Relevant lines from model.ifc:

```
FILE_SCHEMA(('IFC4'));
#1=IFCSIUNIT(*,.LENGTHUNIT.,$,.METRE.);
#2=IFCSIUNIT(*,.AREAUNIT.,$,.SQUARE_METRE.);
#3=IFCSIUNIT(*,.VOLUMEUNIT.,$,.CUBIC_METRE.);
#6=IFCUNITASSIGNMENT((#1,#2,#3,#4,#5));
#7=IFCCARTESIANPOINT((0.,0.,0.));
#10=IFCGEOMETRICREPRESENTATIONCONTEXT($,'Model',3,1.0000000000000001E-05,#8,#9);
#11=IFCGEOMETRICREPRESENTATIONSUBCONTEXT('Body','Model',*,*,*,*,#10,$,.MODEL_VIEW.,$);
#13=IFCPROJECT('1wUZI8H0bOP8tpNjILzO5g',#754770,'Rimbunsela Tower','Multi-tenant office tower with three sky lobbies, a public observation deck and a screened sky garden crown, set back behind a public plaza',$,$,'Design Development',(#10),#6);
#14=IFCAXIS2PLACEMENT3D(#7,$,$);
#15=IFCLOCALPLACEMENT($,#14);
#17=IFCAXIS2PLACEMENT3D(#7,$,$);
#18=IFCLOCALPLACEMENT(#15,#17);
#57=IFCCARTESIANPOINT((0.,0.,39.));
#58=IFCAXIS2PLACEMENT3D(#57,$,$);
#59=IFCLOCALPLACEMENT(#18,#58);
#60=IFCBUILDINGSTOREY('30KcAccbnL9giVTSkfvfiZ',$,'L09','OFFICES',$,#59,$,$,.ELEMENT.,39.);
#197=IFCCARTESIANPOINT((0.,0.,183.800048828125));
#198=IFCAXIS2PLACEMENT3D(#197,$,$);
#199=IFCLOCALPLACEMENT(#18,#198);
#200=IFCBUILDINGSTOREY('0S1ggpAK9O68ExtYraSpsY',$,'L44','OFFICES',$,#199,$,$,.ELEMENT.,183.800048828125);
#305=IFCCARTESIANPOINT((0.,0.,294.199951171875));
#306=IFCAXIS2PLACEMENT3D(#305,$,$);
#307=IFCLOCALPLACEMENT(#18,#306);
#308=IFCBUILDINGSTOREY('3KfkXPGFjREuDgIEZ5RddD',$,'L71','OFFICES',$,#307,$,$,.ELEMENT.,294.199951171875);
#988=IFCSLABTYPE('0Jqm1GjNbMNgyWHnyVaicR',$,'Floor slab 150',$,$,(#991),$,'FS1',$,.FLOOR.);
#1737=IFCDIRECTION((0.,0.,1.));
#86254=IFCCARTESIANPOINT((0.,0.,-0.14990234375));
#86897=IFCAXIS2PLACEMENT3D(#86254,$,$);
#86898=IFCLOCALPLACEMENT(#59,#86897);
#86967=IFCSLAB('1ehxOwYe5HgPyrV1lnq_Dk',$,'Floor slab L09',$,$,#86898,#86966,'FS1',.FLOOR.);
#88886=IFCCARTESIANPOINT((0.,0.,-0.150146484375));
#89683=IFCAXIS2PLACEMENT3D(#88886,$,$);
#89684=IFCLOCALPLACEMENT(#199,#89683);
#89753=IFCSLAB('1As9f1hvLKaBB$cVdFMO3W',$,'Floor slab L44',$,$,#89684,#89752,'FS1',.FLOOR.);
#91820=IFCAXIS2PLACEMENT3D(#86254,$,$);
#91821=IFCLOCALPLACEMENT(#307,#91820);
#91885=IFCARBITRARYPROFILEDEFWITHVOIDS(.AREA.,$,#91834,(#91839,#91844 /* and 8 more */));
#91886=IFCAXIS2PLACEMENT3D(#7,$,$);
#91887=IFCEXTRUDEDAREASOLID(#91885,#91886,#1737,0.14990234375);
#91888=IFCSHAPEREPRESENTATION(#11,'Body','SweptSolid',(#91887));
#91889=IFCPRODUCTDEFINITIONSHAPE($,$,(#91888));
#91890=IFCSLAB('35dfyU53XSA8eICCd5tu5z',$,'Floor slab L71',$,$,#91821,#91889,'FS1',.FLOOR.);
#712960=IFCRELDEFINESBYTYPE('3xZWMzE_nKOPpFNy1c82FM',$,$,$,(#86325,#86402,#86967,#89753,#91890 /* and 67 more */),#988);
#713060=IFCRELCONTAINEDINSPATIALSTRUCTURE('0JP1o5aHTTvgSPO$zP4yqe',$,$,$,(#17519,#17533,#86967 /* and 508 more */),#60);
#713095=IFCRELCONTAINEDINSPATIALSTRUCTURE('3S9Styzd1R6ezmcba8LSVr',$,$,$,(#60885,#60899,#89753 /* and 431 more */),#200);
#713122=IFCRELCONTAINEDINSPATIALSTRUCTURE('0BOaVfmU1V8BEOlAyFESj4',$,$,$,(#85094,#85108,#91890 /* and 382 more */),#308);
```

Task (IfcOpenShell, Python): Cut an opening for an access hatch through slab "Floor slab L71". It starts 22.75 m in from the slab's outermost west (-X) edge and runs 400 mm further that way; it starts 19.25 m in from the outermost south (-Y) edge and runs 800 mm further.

```python
import numpy as np
import ifcopenshell
import ifcopenshell.api.feature
import ifcopenshell.api.geometry
import ifcopenshell.api.root
import ifcopenshell.geom
import ifcopenshell.util.placement
import ifcopenshell.util.representation
import ifcopenshell.util.shape
import ifcopenshell.util.unit

model = ifcopenshell.open("model.ifc")
unit_scale = ifcopenshell.util.unit.calculate_unit_scale(model)
settings = ifcopenshell.geom.settings()


def volume(element):
    """Net volume in cubic metres, openings subtracted."""
    shape = ifcopenshell.geom.create_shape(settings, element)
    return ifcopenshell.util.shape.get_volume(shape.geometry)


slab = model.by_id(91890)
before = volume(slab)

# Extent in the slab's own axes, in metres. The edges named are its -X and -Y sides.
slab_shape = ifcopenshell.geom.create_shape(settings, slab)
vertices = ifcopenshell.util.shape.get_vertices(slab_shape.geometry)
x_min, y_min, bottom = vertices.min(axis=0)
top = vertices[:, 2].max()

opening = ifcopenshell.api.root.create_entity(model, ifc_class="IfcOpeningElement", name="Access hatch opening", predefined_type="OPENING")
context = ifcopenshell.util.representation.get_context(model, "Model", "Body", "MODEL_VIEW")
width, depth = 0.4, 0.8
outline = [(0.0, 0.0), (width, 0.0), (width, depth), (0.0, depth), (0.0, 0.0)]
# Overshoot both faces by 50 mm so the cut is clean.
shape = ifcopenshell.api.geometry.add_slab_representation(
    model, context=context, depth=top - bottom + 0.1, polyline=outline
)
ifcopenshell.api.geometry.assign_representation(model, product=opening, representation=shape)

matrix = ifcopenshell.util.placement.get_local_placement(slab.ObjectPlacement)
matrix[:, 3] = matrix @ np.append(np.array([x_min + 22.75, y_min + 19.25, bottom - 0.05]) / unit_scale, 1.0)
ifcopenshell.api.geometry.edit_object_placement(model, product=opening, matrix=matrix, is_si=False)
ifcopenshell.api.feature.add_feature(model, feature=opening, element=slab)

after = volume(slab)

print(f"slab volume {before:.3f} -> {after:.3f} m3")

model.write("model_rev.ifc")
```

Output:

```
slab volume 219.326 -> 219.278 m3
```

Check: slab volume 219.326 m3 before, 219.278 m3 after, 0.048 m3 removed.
